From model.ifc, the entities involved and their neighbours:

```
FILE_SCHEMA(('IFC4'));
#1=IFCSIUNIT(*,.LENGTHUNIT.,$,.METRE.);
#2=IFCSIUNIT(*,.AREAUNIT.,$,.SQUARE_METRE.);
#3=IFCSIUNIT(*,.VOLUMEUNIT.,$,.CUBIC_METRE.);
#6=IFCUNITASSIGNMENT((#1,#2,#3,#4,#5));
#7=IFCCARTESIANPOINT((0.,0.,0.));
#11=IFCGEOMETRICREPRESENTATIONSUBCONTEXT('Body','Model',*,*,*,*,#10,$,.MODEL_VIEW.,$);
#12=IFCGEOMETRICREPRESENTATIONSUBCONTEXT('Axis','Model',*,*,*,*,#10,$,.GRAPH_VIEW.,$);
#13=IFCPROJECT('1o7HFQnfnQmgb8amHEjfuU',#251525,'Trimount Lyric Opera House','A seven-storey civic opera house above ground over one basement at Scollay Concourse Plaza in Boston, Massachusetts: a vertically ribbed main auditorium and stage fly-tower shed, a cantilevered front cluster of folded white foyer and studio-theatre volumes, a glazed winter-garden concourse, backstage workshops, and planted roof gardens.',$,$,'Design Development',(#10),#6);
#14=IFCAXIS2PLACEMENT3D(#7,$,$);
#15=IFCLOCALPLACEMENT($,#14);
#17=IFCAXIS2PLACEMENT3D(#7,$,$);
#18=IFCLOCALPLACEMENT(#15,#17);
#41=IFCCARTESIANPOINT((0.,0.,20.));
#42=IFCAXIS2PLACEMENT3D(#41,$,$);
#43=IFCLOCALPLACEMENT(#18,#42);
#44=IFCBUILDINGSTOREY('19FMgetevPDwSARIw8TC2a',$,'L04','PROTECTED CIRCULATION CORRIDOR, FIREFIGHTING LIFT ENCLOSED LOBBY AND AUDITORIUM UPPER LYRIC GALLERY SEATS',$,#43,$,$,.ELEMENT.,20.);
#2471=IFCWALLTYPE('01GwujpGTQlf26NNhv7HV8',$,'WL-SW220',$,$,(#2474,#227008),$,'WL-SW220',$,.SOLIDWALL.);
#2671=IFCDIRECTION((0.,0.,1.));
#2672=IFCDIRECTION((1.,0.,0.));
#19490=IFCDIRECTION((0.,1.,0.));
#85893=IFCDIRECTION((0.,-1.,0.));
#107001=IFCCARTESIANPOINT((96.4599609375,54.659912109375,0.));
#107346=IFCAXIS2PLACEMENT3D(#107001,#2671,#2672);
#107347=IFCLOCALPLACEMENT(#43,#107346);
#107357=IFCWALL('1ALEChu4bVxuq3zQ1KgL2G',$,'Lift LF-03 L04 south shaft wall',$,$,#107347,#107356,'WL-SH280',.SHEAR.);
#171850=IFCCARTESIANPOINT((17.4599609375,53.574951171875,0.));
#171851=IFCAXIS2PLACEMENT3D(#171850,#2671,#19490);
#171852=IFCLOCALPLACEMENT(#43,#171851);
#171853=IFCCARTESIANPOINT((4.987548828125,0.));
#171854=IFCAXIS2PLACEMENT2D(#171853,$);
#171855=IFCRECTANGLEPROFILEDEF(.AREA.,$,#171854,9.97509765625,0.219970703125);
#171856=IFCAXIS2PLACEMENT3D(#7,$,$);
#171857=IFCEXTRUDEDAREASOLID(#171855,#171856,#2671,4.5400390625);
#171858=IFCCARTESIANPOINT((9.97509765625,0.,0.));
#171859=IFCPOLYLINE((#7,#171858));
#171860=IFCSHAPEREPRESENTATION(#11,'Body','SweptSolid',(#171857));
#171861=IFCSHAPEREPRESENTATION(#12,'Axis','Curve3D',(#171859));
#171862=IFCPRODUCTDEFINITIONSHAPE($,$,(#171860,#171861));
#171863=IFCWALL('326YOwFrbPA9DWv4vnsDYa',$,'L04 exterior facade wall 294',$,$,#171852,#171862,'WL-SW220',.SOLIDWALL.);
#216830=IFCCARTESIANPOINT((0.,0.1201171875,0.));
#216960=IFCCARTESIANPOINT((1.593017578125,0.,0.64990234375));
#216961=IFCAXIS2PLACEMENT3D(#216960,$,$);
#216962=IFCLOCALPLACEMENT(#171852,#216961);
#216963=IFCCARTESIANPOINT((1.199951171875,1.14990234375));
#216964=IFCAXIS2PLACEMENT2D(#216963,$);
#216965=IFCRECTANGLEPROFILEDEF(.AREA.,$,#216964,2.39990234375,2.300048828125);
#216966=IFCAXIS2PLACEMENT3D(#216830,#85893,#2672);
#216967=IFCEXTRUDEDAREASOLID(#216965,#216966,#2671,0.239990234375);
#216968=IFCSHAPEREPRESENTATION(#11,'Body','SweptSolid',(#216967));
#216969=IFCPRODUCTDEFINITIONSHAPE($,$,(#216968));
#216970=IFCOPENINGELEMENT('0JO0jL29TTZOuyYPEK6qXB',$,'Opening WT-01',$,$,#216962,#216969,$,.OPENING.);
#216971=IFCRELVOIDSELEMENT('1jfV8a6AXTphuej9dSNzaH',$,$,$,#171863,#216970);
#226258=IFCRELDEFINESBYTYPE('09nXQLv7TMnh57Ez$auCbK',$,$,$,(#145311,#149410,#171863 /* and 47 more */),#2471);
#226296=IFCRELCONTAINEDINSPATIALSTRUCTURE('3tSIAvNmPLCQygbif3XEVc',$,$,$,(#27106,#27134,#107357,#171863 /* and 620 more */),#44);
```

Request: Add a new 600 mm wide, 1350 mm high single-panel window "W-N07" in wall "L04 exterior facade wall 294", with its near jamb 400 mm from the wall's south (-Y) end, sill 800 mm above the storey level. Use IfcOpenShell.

```python
import numpy as np
import ifcopenshell
import ifcopenshell.api.feature
import ifcopenshell.api.geometry
import ifcopenshell.api.root
import ifcopenshell.api.spatial
import ifcopenshell.geom
import ifcopenshell.util.element
import ifcopenshell.util.placement
import ifcopenshell.util.representation
import ifcopenshell.util.shape
import ifcopenshell.util.unit

model = ifcopenshell.open("model.ifc")
unit_scale = ifcopenshell.util.unit.calculate_unit_scale(model)
settings = ifcopenshell.geom.settings()


def volume(element):
    """Net volume in cubic metres, openings subtracted."""
    shape = ifcopenshell.geom.create_shape(settings, element)
    return ifcopenshell.util.shape.get_volume(shape.geometry)


wall = model.by_id(171863)
storey = ifcopenshell.util.element.get_container(wall, ifc_class="IfcBuildingStorey")
context = ifcopenshell.util.representation.get_context(model, "Model", "Body", "MODEL_VIEW")
before = volume(wall)

width, height, from_end, sill = 0.6, 1.35, 0.4, 0.8  # metres

# The wall runs along its own X axis, and the end named is its -X end.
wall_shape = ifcopenshell.geom.create_shape(settings, wall)
x, y, z = ifcopenshell.util.shape.get_vertices(wall_shape.geometry).T
start = x.min() + from_end
face, thickness = float(y.min()), float(y.max() - y.min())
wall_matrix = ifcopenshell.util.placement.get_local_placement(wall.ObjectPlacement)
level = ifcopenshell.util.placement.get_local_placement(storey.ObjectPlacement)[2, 3]


def in_wall(x, y):
    """Placement at x, y metres in the wall's axes, at sill height."""
    matrix = wall_matrix.copy()
    matrix[:, 3] = wall_matrix @ np.array([x / unit_scale, y / unit_scale, 0.0, 1.0])
    matrix[2, 3] = level + sill / unit_scale
    return matrix


# Opening: a box that overshoots both wall faces by 50 mm.
opening = ifcopenshell.api.root.create_entity(model, ifc_class="IfcOpeningElement", predefined_type="OPENING")
box = ifcopenshell.api.geometry.add_wall_representation(
    model, context=context, length=width, height=height, thickness=thickness + 0.1
)
ifcopenshell.api.geometry.assign_representation(model, product=opening, representation=box)
ifcopenshell.api.geometry.edit_object_placement(model, product=opening, matrix=in_wall(start, face - 0.05), is_si=False)
ifcopenshell.api.feature.add_feature(model, feature=opening, element=wall)

window = ifcopenshell.api.root.create_entity(model, ifc_class="IfcWindow", name="W-N07", predefined_type="WINDOW")
window.OverallWidth, window.OverallHeight = width / unit_scale, height / unit_scale
window.PartitioningType = "SINGLE_PANEL"
body = ifcopenshell.api.geometry.add_window_representation(
    model,
    context=context,
    overall_width=window.OverallWidth,
    overall_height=window.OverallHeight,
    partition_type="SINGLE_PANEL",
)
ifcopenshell.api.geometry.assign_representation(model, product=window, representation=body)
ifcopenshell.api.spatial.assign_container(model, products=[window], relating_structure=storey)
ifcopenshell.api.feature.add_filling(model, opening=opening, element=window)

# Centre the window in the wall's thickness.
ifcopenshell.api.geometry.edit_object_placement(model, product=window, matrix=in_wall(start, face), is_si=False)
window_shape = ifcopenshell.geom.create_shape(settings, window)
depth = ifcopenshell.util.shape.get_vertices(window_shape.geometry)[:, 1]
offset = face + thickness / 2 - (depth.min() + depth.max()) / 2
ifcopenshell.api.geometry.edit_object_placement(model, product=window, matrix=in_wall(start, offset), is_si=False)

after = volume(wall)

print(f"wall volume {before:.3f} -> {after:.3f} m3")

model.write("model_v2.ifc")
```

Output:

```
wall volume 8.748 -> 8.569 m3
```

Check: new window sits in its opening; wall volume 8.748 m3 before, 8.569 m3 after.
